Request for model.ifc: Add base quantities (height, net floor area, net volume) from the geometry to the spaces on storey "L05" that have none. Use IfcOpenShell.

First a look at what the model holds.

```python
import ifcopenshell
import ifcopenshell.util.element
import ifcopenshell.util.unit

model = ifcopenshell.open("model.ifc")
print(model.schema)
for unit_type in ("LENGTHUNIT", "AREAUNIT", "VOLUMEUNIT"):
    print(unit_type, ifcopenshell.util.unit.calculate_unit_scale(model, unit_type))
storey = next(s for s in model.by_type("IfcBuildingStorey") if s.Name == "L05")
spaces = [e for e in ifcopenshell.util.element.get_decomposition(storey) if e.is_a("IfcSpace")]
for e in sorted(spaces, key=lambda e: e.id()):
    print(e.id(), e.is_a(), e.Name, list(ifcopenshell.util.element.get_psets(e, qtos_only=True)), sep=" | ")
```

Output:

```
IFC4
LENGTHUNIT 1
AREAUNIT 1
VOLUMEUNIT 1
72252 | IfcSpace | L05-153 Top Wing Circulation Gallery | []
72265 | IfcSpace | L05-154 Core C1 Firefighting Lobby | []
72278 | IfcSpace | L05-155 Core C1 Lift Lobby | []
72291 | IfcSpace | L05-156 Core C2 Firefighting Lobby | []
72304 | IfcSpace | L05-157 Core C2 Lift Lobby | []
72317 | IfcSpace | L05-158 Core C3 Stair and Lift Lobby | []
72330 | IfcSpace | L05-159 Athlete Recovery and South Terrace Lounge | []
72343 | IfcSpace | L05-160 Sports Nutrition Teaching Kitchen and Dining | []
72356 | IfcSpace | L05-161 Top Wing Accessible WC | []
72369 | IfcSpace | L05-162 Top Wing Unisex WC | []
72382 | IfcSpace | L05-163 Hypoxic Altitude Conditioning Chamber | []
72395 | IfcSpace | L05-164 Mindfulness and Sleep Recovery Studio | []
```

```python
import ifcopenshell
import ifcopenshell.api.pset
import ifcopenshell.geom
import ifcopenshell.util.element
import ifcopenshell.util.shape
import ifcopenshell.util.unit

model = ifcopenshell.open("model.ifc")
unit_scale = ifcopenshell.util.unit.calculate_unit_scale(model)
area_scale = ifcopenshell.util.unit.calculate_unit_scale(model, "AREAUNIT")
volume_scale = ifcopenshell.util.unit.calculate_unit_scale(model, "VOLUMEUNIT")
settings = ifcopenshell.geom.settings()

storey = next(s for s in model.by_type("IfcBuildingStorey") if s.Name == "L05")
spaces = [e for e in ifcopenshell.util.element.get_decomposition(storey) if e.is_a("IfcSpace")]

for e in sorted(spaces, key=lambda e: e.id()):
    if ifcopenshell.util.element.get_psets(e, qtos_only=True, should_inherit=False):
        continue
    # Geometry comes back in metres, in the element's own axes.
    shape = ifcopenshell.geom.create_shape(settings, e)
    values = {
        "Height": ifcopenshell.util.shape.get_z(shape.geometry) / unit_scale,
        "NetFloorArea": ifcopenshell.util.shape.get_footprint_area(shape.geometry) / area_scale,
        "NetVolume": ifcopenshell.util.shape.get_volume(shape.geometry) / volume_scale,
    }
    qto = ifcopenshell.api.pset.add_qto(model, product=e, name="Qto_SpaceBaseQuantities")
    ifcopenshell.api.pset.edit_qto(model, qto=qto, properties=values)
    print(e.id(), {k: round(v, 3) for k, v in values.items()})

model.write("model_edited.ifc")
```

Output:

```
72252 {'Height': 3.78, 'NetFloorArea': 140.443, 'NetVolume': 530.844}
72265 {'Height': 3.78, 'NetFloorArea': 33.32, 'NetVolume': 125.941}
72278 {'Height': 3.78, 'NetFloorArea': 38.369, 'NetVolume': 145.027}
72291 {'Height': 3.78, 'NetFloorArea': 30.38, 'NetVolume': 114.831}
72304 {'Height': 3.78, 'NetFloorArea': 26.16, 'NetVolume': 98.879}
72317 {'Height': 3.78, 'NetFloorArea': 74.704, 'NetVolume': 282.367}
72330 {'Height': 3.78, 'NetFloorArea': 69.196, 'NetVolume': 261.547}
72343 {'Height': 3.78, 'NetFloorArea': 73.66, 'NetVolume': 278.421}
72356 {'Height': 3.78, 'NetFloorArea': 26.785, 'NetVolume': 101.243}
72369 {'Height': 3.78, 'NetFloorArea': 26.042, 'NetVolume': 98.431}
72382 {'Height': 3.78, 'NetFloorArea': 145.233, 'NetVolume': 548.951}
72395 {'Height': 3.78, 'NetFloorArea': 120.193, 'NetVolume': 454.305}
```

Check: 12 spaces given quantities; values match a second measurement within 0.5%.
